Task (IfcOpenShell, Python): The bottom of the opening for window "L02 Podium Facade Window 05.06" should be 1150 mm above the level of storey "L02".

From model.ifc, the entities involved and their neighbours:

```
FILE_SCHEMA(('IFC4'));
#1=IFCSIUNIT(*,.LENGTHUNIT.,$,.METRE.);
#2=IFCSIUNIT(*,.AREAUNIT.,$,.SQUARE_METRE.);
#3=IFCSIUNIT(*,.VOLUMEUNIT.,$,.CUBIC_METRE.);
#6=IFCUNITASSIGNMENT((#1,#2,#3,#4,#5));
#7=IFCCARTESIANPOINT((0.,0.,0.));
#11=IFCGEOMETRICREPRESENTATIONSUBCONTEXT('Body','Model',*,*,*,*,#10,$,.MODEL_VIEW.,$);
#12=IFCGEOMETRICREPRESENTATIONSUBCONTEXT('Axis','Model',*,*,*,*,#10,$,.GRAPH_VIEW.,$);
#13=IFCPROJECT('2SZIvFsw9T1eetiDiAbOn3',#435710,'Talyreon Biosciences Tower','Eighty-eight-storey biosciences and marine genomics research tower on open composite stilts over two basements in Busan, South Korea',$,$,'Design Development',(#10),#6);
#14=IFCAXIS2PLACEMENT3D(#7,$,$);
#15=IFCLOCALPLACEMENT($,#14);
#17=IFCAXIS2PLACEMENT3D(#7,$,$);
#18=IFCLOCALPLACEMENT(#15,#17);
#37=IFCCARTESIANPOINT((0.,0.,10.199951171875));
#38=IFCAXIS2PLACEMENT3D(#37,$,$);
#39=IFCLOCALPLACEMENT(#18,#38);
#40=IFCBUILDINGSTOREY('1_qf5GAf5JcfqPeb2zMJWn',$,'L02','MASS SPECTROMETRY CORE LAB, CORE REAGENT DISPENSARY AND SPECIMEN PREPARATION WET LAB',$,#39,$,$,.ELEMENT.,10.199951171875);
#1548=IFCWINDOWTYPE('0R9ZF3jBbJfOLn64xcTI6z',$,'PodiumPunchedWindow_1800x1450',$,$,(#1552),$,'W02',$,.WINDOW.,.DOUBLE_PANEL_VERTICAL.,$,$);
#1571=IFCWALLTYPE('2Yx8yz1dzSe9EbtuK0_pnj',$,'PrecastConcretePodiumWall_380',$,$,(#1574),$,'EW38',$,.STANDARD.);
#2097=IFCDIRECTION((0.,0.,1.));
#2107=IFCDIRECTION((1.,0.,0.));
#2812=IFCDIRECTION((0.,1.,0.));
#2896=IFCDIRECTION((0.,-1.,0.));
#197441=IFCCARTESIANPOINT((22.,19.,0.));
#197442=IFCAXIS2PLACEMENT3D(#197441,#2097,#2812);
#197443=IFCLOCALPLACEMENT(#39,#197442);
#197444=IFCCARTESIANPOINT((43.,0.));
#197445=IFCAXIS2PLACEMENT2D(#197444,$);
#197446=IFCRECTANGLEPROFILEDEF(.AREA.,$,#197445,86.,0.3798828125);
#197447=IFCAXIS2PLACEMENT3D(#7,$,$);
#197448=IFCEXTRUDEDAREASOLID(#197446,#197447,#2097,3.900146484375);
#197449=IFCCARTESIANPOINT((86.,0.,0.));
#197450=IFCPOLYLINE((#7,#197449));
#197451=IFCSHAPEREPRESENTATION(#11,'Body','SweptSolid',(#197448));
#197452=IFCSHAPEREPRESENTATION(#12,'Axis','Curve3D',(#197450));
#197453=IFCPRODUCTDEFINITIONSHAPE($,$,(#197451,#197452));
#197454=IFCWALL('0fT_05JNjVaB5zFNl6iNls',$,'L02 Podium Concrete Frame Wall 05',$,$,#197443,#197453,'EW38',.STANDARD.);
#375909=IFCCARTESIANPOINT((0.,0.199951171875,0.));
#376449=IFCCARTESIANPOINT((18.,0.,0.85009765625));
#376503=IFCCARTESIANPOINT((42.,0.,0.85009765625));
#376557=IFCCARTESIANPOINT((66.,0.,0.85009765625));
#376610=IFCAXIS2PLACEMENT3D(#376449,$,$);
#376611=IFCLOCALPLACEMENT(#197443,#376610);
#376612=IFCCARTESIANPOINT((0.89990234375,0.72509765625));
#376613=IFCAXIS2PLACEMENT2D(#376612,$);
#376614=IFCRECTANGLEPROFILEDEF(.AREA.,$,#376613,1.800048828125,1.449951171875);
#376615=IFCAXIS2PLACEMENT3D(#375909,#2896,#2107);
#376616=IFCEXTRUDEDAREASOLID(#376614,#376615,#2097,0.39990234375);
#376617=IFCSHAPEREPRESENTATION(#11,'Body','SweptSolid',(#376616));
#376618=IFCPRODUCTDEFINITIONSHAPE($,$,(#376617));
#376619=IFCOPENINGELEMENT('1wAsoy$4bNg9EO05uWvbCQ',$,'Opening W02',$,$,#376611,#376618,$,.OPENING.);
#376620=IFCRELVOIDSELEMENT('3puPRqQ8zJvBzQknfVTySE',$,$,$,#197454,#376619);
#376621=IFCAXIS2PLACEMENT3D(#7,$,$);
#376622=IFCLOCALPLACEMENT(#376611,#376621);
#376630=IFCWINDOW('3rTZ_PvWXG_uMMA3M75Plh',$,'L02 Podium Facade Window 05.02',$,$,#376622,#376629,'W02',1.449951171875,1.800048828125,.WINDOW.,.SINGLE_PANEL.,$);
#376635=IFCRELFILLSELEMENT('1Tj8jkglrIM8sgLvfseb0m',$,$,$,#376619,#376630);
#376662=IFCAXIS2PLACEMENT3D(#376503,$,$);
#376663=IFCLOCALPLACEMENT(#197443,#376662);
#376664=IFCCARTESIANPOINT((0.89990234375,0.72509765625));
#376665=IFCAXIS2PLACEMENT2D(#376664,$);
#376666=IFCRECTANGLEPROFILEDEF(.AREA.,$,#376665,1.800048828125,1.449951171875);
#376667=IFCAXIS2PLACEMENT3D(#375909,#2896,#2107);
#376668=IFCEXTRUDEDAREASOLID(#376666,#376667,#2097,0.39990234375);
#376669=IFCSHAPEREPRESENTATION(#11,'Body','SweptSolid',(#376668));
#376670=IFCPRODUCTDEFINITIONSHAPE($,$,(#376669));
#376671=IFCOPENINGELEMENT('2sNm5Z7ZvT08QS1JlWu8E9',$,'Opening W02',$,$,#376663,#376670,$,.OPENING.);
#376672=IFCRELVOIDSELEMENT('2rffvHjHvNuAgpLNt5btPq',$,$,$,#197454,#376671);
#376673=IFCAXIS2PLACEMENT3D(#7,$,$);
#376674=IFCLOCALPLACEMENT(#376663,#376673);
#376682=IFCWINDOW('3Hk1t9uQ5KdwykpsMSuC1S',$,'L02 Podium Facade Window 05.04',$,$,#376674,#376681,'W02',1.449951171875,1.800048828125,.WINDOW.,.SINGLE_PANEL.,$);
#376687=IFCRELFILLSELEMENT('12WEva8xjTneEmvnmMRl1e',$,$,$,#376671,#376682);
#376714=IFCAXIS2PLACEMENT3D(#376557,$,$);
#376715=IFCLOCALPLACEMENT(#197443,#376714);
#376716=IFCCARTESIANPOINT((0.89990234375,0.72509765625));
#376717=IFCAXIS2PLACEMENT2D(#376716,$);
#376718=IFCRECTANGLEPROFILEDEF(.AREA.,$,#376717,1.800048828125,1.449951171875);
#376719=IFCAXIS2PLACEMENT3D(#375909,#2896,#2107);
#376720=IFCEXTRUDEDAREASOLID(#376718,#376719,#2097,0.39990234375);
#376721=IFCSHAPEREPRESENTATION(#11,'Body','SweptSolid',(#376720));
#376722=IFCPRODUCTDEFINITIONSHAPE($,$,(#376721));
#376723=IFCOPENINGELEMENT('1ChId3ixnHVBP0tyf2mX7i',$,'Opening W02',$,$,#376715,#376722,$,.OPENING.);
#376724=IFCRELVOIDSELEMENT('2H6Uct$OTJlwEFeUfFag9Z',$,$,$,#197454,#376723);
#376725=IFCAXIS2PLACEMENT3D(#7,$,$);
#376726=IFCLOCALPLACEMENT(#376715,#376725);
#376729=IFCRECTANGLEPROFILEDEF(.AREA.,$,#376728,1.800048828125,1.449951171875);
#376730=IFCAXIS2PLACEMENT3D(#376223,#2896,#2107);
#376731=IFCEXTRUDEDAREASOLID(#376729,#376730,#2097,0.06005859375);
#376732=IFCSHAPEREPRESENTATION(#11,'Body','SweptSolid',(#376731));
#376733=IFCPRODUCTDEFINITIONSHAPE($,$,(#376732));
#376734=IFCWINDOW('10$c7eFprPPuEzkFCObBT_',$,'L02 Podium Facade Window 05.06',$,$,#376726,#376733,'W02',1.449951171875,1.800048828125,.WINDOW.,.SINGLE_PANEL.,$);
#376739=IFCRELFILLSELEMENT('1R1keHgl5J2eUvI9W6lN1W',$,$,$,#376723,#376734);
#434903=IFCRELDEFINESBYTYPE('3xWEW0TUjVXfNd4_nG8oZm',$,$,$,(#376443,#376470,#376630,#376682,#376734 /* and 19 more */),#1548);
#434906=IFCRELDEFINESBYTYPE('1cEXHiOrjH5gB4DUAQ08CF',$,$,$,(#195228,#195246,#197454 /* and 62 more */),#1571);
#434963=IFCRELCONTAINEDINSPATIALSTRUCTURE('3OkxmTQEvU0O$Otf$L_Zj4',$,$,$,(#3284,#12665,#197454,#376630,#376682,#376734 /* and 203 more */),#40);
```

```python
import numpy as np
import ifcopenshell
import ifcopenshell.api.geometry
import ifcopenshell.geom
import ifcopenshell.util.element
import ifcopenshell.util.placement
import ifcopenshell.util.shape
import ifcopenshell.util.unit

model = ifcopenshell.open("model.ifc")
unit_scale = ifcopenshell.util.unit.calculate_unit_scale(model)

window = model.by_guid("10$c7eFprPPuEzkFCObBT_")
opening = window.FillsVoids[0].RelatingOpeningElement
storey = ifcopenshell.util.element.get_container(window, ifc_class="IfcBuildingStorey")
level = ifcopenshell.util.placement.get_local_placement(storey.ObjectPlacement)[2, 3]

# The opening's origin need not be at the sill, so measure its lowest point.
shape = ifcopenshell.geom.create_shape(ifcopenshell.geom.settings(), opening)
bottom = ifcopenshell.util.shape.get_shape_bottom_elevation(shape, shape.geometry) / unit_scale
dz = level + 1.15 / unit_scale - bottom

shift = np.array([0.0, 0.0, dz])
# The window is placed relative to its opening, so it follows when the opening moves.
matrix = ifcopenshell.util.placement.get_local_placement(opening.ObjectPlacement)
matrix[:3, 3] += shift
ifcopenshell.api.geometry.edit_object_placement(
    model, product=opening, matrix=matrix, is_si=False, should_transform_children=True
)

print(f"moved by {dz * unit_scale:+.3f} m")

model.write("model-out.ifc")
```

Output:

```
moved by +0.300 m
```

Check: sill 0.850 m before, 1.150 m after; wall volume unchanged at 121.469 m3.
